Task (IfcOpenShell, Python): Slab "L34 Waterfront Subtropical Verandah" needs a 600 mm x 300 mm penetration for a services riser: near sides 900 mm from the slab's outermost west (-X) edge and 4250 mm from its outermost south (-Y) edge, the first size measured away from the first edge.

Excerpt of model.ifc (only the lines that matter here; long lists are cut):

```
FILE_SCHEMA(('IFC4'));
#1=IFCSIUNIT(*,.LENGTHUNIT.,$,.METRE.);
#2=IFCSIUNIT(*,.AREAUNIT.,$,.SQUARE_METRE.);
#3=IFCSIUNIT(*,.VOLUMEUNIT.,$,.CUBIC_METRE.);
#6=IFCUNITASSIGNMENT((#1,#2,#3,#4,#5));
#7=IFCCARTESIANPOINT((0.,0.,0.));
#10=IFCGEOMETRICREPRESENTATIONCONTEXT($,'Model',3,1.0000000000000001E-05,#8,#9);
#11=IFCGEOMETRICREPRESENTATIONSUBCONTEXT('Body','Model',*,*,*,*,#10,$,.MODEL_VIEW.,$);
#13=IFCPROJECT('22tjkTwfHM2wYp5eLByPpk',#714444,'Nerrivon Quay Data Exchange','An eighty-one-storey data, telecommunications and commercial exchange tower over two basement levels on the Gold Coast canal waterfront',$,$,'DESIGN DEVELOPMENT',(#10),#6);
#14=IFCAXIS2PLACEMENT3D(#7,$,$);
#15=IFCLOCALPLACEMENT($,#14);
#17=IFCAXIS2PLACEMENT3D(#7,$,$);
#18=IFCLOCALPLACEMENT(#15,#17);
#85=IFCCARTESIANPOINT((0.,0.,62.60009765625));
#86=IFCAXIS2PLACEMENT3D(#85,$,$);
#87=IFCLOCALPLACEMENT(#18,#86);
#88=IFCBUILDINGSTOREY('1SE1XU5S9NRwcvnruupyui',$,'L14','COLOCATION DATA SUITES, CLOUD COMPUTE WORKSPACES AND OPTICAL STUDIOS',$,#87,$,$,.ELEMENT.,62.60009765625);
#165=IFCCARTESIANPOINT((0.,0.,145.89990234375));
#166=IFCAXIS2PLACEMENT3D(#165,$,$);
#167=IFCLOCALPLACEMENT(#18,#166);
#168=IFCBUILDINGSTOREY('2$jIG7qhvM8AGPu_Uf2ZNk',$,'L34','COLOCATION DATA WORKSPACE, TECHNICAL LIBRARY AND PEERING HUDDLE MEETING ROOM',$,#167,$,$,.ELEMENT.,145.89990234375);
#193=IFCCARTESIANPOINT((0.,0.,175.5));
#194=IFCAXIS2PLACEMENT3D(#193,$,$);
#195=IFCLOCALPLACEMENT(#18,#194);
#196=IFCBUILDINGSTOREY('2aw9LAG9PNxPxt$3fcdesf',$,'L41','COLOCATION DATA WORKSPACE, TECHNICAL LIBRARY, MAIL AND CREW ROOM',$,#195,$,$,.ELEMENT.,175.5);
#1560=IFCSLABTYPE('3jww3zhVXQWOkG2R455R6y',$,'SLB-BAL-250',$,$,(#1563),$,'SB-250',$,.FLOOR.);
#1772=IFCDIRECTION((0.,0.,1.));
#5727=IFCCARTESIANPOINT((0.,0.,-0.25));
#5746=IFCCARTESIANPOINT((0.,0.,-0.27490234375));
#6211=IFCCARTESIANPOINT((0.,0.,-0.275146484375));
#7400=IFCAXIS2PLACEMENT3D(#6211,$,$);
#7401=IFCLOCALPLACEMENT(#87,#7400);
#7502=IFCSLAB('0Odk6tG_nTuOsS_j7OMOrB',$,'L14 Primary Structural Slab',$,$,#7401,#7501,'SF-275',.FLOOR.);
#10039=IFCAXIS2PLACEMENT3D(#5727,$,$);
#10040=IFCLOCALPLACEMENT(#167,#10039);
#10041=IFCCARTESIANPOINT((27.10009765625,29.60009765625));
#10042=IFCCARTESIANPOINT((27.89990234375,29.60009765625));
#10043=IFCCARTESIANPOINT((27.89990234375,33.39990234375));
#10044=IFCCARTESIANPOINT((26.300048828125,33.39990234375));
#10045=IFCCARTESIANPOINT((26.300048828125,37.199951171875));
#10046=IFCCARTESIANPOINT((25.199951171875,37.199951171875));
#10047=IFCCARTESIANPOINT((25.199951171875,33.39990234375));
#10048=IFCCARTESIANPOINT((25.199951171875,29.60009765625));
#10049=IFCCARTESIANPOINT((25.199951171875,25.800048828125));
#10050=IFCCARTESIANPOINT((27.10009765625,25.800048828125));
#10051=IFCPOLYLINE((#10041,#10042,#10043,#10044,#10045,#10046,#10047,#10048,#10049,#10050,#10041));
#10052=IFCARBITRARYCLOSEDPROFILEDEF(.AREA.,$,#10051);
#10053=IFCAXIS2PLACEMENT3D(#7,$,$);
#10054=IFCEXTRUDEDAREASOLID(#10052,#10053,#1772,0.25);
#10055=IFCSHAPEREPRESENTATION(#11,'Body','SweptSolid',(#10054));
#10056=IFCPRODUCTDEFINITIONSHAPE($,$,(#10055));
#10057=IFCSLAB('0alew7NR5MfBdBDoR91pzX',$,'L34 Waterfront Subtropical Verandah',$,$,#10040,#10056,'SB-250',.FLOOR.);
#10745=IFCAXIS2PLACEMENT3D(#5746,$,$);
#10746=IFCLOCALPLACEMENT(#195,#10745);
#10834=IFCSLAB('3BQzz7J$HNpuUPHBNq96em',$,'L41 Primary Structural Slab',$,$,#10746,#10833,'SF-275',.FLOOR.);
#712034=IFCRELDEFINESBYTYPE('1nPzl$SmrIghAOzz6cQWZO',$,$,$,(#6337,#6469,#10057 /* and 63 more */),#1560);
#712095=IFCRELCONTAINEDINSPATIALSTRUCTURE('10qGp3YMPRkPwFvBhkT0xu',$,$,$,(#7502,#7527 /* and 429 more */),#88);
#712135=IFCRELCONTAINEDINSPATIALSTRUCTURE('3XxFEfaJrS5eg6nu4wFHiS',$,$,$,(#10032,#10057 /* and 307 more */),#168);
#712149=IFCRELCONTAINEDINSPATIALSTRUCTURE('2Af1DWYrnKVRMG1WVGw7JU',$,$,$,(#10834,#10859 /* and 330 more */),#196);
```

```python
import numpy as np
import ifcopenshell
import ifcopenshell.api.feature
import ifcopenshell.api.geometry
import ifcopenshell.api.root
import ifcopenshell.geom
import ifcopenshell.util.placement
import ifcopenshell.util.representation
import ifcopenshell.util.shape
import ifcopenshell.util.unit

model = ifcopenshell.open("model.ifc")
unit_scale = ifcopenshell.util.unit.calculate_unit_scale(model)
settings = ifcopenshell.geom.settings()


def volume(element):
    """Net volume in cubic metres, openings subtracted."""
    shape = ifcopenshell.geom.create_shape(settings, element)
    return ifcopenshell.util.shape.get_volume(shape.geometry)


slab = model.by_guid("0alew7NR5MfBdBDoR91pzX")
before = volume(slab)

# Extent in the slab's own axes, in metres. The edges named are its -X and -Y sides.
slab_shape = ifcopenshell.geom.create_shape(settings, slab)
vertices = ifcopenshell.util.shape.get_vertices(slab_shape.geometry)
x_min, y_min, bottom = vertices.min(axis=0)
top = vertices[:, 2].max()

opening = ifcopenshell.api.root.create_entity(model, ifc_class="IfcOpeningElement", name="Services riser opening", predefined_type="OPENING")
context = ifcopenshell.util.representation.get_context(model, "Model", "Body", "MODEL_VIEW")
width, depth = 0.6, 0.3
outline = [(0.0, 0.0), (width, 0.0), (width, depth), (0.0, depth), (0.0, 0.0)]
# Overshoot both faces by 50 mm so the cut is clean.
shape = ifcopenshell.api.geometry.add_slab_representation(
    model, context=context, depth=top - bottom + 0.1, polyline=outline
)
ifcopenshell.api.geometry.assign_representation(model, product=opening, representation=shape)

matrix = ifcopenshell.util.placement.get_local_placement(slab.ObjectPlacement)
matrix[:, 3] = matrix @ np.append(np.array([x_min + 0.9, y_min + 4.25, bottom - 0.05]) / unit_scale, 1.0)
ifcopenshell.api.geometry.edit_object_placement(model, product=opening, matrix=matrix, is_si=False)
ifcopenshell.api.feature.add_feature(model, feature=opening, element=slab)

after = volume(slab)

print(f"slab volume {before:.3f} -> {after:.3f} m3")

model.write("model-out.ifc")
```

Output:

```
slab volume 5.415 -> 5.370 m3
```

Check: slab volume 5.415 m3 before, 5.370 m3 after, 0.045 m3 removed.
